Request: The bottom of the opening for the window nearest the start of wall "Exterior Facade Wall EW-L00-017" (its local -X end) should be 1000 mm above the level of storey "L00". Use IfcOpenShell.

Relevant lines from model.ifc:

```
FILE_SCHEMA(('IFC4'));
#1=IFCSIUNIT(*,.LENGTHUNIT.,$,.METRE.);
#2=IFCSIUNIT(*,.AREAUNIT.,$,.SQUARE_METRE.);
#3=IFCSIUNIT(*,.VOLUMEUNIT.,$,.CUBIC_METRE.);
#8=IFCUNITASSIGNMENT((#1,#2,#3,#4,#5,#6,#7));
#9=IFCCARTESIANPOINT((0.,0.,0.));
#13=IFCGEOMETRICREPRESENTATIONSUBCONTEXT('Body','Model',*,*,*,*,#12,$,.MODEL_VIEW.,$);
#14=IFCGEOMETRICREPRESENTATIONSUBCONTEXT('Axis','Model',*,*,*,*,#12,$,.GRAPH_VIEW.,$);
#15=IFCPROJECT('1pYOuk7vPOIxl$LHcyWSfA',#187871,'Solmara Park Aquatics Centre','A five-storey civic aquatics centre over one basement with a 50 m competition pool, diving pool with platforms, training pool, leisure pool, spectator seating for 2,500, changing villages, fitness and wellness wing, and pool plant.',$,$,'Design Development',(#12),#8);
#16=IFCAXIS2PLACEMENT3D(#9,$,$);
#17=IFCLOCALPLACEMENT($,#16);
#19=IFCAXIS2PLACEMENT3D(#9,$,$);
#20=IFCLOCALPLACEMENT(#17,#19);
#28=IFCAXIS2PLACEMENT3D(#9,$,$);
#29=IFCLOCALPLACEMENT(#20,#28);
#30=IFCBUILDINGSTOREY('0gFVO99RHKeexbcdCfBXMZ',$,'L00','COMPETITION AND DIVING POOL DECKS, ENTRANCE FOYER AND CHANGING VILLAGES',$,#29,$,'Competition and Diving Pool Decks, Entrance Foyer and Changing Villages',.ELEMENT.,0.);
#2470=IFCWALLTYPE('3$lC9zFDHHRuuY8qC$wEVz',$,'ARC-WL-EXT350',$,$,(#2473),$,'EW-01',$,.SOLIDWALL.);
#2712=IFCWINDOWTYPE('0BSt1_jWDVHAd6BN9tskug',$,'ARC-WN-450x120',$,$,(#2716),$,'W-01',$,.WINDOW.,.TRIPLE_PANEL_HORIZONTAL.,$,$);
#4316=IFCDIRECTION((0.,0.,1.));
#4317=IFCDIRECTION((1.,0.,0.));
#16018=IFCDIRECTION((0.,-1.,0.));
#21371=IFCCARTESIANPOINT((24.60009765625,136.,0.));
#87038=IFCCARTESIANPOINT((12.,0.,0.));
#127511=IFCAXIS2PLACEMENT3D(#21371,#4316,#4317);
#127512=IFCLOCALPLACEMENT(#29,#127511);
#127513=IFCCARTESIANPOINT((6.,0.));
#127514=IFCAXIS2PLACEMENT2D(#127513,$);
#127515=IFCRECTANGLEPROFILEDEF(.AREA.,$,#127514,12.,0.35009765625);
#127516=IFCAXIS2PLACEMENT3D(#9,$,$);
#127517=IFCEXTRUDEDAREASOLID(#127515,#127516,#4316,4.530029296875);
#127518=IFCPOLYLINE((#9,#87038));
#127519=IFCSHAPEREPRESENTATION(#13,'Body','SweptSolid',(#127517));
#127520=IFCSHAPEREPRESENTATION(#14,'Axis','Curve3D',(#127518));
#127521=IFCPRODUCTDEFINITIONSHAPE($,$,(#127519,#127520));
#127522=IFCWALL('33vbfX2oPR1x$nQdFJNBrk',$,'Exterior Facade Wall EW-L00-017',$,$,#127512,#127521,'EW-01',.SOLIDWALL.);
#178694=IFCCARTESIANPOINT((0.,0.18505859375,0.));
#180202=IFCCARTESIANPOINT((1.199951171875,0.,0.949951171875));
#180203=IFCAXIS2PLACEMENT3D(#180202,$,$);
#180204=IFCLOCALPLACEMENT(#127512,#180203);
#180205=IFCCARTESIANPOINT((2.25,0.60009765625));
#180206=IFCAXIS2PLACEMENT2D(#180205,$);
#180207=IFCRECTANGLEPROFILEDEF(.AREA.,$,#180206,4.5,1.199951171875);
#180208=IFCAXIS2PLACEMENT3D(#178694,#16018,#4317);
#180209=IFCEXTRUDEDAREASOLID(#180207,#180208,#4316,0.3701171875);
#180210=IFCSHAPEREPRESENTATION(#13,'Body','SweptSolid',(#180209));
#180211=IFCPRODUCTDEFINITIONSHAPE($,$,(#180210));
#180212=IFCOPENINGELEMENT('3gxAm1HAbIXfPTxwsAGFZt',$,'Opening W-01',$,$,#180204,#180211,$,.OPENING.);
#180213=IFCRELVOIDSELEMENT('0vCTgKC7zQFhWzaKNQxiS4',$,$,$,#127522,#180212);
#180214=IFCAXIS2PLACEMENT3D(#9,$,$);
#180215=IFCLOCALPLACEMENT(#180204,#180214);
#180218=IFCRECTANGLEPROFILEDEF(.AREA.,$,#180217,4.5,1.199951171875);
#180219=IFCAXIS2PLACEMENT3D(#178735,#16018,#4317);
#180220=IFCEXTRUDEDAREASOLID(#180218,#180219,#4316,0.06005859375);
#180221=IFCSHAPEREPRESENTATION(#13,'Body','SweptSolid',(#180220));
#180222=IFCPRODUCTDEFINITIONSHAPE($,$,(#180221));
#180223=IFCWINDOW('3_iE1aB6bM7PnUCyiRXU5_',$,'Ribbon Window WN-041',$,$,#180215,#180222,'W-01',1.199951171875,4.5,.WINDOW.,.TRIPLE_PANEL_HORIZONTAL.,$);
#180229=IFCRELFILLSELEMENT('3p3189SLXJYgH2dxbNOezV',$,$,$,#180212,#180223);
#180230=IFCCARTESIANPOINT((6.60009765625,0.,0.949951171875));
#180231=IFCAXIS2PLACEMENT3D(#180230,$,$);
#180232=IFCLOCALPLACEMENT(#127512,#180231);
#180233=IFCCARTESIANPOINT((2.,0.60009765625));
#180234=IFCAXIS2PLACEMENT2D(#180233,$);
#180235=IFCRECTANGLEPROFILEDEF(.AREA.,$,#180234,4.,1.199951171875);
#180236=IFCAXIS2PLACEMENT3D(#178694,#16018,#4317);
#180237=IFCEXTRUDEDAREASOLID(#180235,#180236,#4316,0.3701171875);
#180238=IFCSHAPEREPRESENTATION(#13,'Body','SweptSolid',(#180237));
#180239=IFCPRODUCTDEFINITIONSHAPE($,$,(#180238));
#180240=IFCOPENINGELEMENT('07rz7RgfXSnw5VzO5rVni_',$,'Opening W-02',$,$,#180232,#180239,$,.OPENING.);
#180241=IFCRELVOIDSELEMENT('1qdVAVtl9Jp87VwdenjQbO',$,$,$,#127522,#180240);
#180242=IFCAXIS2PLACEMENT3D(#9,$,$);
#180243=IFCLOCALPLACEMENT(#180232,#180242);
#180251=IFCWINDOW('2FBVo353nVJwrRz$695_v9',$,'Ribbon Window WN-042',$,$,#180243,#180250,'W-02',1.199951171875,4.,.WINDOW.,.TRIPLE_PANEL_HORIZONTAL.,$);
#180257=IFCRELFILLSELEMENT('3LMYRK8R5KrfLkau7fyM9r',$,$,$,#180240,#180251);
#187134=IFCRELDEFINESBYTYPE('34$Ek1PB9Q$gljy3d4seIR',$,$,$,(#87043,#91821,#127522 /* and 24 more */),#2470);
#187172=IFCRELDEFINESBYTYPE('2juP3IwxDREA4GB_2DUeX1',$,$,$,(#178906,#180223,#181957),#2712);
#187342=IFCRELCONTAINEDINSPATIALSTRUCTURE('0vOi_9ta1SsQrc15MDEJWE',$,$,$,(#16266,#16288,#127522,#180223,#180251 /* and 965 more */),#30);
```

```python
import numpy as np
import ifcopenshell
import ifcopenshell.api.geometry
import ifcopenshell.geom
import ifcopenshell.util.element
import ifcopenshell.util.placement
import ifcopenshell.util.shape
import ifcopenshell.util.unit

model = ifcopenshell.open("model.ifc")
unit_scale = ifcopenshell.util.unit.calculate_unit_scale(model)

window = model.by_guid("3_iE1aB6bM7PnUCyiRXU5_")
opening = window.FillsVoids[0].RelatingOpeningElement
storey = ifcopenshell.util.element.get_container(window, ifc_class="IfcBuildingStorey")
level = ifcopenshell.util.placement.get_local_placement(storey.ObjectPlacement)[2, 3]

# The opening's origin need not be at the sill, so measure its lowest point.
shape = ifcopenshell.geom.create_shape(ifcopenshell.geom.settings(), opening)
bottom = ifcopenshell.util.shape.get_shape_bottom_elevation(shape, shape.geometry) / unit_scale
dz = level + 1 / unit_scale - bottom

shift = np.array([0.0, 0.0, dz])
# The window is placed relative to its opening, so it follows when the opening moves.
matrix = ifcopenshell.util.placement.get_local_placement(opening.ObjectPlacement)
matrix[:3, 3] += shift
ifcopenshell.api.geometry.edit_object_placement(
    model, product=opening, matrix=matrix, is_si=False, should_transform_children=True
)

print(f"moved by {dz * unit_scale:+.3f} m")

model.write("model-out.ifc")
```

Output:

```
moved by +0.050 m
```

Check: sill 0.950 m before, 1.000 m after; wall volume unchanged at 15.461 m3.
